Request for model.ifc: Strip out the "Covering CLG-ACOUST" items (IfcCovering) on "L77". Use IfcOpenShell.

First a look at what the model holds.

```python
import ifcopenshell
import ifcopenshell.util.element

model = ifcopenshell.open("model.ifc")
print(model.schema)
storey = next(s for s in model.by_type("IfcBuildingStorey") if s.Name == "L77")
coverings = [e for e in ifcopenshell.util.element.get_decomposition(storey) if e.is_a("IfcCovering")]
seen = {}
for e in coverings:
    element_type = ifcopenshell.util.element.get_type(e)
    name = element_type.Name if element_type not in (None, e) else None
    seen[name] = seen.get(name, 0) + 1
for name, count in sorted(seen.items(), key=str):
    print(count, "x", name)
```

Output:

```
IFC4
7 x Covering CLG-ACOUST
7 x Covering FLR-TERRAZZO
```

```python
import ifcopenshell
import ifcopenshell.api.root
import ifcopenshell.util.element

model = ifcopenshell.open("model.ifc")

storey = next(s for s in model.by_type("IfcBuildingStorey") if s.Name == "L77")
coverings = [e for e in ifcopenshell.util.element.get_decomposition(storey) if e.is_a("IfcCovering")]
targets = [e for e in coverings if (t := ifcopenshell.util.element.get_type(e)) not in (None, e) and t.Name == "Covering CLG-ACOUST"]

for e in targets:
    ifcopenshell.api.root.remove_product(model, product=e)
print(len(targets), "removed")

model.write("model_rev.ifc")
```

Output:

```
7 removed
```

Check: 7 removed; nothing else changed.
